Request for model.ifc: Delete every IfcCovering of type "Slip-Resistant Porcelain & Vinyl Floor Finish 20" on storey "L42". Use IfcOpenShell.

First a look at what the model holds.

```python
import ifcopenshell
import ifcopenshell.util.element

model = ifcopenshell.open("model.ifc")
print(model.schema)
storey = next(s for s in model.by_type("IfcBuildingStorey") if s.Name == "L42")
coverings = [e for e in ifcopenshell.util.element.get_decomposition(storey) if e.is_a("IfcCovering")]
seen = {}
for e in coverings:
    element_type = ifcopenshell.util.element.get_type(e)
    name = element_type.Name if element_type not in (None, e) else None
    seen[name] = seen.get(name, 0) + 1
for name, count in sorted(seen.items(), key=str):
    print(count, "x", name)
```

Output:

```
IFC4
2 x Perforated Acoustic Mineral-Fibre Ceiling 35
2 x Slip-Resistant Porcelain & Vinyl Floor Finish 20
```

```python
import ifcopenshell
import ifcopenshell.api.root
import ifcopenshell.util.element

model = ifcopenshell.open("model.ifc")

storey = next(s for s in model.by_type("IfcBuildingStorey") if s.Name == "L42")
coverings = [e for e in ifcopenshell.util.element.get_decomposition(storey) if e.is_a("IfcCovering")]
targets = [e for e in coverings if (t := ifcopenshell.util.element.get_type(e)) not in (None, e) and t.Name == "Slip-Resistant Porcelain & Vinyl Floor Finish 20"]

for e in targets:
    ifcopenshell.api.root.remove_product(model, product=e)
print(len(targets), "removed")

model.write("model-out.ifc")
```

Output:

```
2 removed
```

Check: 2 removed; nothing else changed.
